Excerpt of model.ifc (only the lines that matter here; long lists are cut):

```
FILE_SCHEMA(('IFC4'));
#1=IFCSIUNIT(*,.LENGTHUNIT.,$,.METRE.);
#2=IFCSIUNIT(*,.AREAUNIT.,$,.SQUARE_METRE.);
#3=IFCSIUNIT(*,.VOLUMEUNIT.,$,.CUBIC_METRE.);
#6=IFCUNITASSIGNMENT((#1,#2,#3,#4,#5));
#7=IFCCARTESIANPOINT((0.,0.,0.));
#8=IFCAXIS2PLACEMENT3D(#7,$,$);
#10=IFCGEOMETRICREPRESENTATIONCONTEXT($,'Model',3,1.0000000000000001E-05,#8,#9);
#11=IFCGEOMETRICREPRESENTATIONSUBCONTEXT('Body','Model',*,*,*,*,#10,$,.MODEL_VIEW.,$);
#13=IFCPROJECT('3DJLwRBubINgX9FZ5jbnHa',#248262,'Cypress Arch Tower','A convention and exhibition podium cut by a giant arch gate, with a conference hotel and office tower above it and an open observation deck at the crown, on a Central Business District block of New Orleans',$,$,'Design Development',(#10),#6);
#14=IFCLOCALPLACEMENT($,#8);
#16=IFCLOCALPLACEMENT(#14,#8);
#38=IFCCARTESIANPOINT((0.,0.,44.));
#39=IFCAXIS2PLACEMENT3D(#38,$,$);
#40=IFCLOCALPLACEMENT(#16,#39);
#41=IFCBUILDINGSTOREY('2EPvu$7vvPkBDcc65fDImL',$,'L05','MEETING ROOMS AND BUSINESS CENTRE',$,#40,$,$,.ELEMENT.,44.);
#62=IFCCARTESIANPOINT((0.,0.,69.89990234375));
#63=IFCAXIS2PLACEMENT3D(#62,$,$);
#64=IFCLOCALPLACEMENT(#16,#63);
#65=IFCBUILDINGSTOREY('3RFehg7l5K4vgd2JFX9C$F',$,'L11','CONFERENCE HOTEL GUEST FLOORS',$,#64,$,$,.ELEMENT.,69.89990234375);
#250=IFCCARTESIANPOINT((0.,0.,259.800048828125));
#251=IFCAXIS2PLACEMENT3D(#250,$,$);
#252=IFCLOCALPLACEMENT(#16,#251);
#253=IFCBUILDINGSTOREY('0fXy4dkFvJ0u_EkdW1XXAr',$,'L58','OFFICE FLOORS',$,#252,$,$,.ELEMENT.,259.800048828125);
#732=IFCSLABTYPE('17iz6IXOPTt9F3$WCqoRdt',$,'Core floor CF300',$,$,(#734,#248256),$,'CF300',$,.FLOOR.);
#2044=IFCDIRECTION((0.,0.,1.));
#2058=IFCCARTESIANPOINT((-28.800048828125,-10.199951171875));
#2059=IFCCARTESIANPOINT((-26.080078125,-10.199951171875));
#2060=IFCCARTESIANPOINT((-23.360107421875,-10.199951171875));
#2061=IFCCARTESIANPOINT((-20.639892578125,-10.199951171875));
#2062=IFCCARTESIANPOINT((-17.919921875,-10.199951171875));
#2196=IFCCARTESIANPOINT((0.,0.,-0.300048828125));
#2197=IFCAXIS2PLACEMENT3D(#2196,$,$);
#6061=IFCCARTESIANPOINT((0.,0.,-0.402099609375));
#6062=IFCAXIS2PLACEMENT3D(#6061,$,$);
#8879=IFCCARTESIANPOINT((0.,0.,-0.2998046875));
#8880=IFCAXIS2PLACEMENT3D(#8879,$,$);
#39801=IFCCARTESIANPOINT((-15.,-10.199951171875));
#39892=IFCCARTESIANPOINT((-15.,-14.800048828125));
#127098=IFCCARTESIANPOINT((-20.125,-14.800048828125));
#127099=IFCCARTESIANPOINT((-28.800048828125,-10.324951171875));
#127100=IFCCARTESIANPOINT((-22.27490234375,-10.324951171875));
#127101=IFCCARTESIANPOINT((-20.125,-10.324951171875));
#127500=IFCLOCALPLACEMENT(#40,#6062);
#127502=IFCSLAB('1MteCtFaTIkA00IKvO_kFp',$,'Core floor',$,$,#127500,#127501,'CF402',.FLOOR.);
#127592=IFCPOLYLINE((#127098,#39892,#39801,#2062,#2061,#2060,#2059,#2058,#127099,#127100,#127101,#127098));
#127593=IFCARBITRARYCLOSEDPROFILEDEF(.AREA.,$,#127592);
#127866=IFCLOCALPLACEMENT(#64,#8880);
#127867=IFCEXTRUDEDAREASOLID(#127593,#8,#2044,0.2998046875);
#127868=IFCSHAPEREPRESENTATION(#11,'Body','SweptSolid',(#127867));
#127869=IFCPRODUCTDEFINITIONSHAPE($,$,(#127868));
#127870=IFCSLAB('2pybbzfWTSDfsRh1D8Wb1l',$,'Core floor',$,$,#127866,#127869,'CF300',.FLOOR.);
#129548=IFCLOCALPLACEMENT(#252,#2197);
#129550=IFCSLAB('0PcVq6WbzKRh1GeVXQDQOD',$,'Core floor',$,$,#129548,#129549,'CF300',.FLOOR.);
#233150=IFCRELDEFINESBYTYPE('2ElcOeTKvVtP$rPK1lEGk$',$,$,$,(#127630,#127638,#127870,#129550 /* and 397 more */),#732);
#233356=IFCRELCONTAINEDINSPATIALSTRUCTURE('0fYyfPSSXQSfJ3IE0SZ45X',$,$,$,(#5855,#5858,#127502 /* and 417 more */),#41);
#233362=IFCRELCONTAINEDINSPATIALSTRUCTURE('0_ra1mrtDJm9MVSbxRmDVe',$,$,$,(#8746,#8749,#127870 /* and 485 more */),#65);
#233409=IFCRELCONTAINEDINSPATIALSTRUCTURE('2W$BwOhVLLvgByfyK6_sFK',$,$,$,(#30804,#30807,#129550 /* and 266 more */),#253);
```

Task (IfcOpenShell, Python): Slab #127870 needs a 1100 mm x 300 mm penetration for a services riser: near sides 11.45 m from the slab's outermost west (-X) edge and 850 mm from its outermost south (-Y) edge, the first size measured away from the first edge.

```python
import numpy as np
import ifcopenshell
import ifcopenshell.api.feature
import ifcopenshell.api.geometry
import ifcopenshell.api.root
import ifcopenshell.geom
import ifcopenshell.util.placement
import ifcopenshell.util.representation
import ifcopenshell.util.shape
import ifcopenshell.util.unit

model = ifcopenshell.open("model.ifc")
unit_scale = ifcopenshell.util.unit.calculate_unit_scale(model)
settings = ifcopenshell.geom.settings()


def volume(element):
    """Net volume in cubic metres, openings subtracted."""
    shape = ifcopenshell.geom.create_shape(settings, element)
    return ifcopenshell.util.shape.get_volume(shape.geometry)


slab = model.by_id(127870)
before = volume(slab)

# Extent in the slab's own axes, in metres. The edges named are its -X and -Y sides.
slab_shape = ifcopenshell.geom.create_shape(settings, slab)
vertices = ifcopenshell.util.shape.get_vertices(slab_shape.geometry)
x_min, y_min, bottom = vertices.min(axis=0)
top = vertices[:, 2].max()

opening = ifcopenshell.api.root.create_entity(model, ifc_class="IfcOpeningElement", name="Services riser opening", predefined_type="OPENING")
context = ifcopenshell.util.representation.get_context(model, "Model", "Body", "MODEL_VIEW")
width, depth = 1.1, 0.3
outline = [(0.0, 0.0), (width, 0.0), (width, depth), (0.0, depth), (0.0, 0.0)]
# Overshoot both faces by 50 mm so the cut is clean.
shape = ifcopenshell.api.geometry.add_slab_representation(
    model, context=context, depth=top - bottom + 0.1, polyline=outline
)
ifcopenshell.api.geometry.assign_representation(model, product=opening, representation=shape)

matrix = ifcopenshell.util.placement.get_local_placement(slab.ObjectPlacement)
matrix[:, 3] = matrix @ np.append(np.array([x_min + 11.45, y_min + 0.85, bottom - 0.05]) / unit_scale, 1.0)
ifcopenshell.api.geometry.edit_object_placement(model, product=opening, matrix=matrix, is_si=False)
ifcopenshell.api.feature.add_feature(model, feature=opening, element=slab)

after = volume(slab)

print(f"slab volume {before:.3f} -> {after:.3f} m3")

model.write("model_v2.ifc")
```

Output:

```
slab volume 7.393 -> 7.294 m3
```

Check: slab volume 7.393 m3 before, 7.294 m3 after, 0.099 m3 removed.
